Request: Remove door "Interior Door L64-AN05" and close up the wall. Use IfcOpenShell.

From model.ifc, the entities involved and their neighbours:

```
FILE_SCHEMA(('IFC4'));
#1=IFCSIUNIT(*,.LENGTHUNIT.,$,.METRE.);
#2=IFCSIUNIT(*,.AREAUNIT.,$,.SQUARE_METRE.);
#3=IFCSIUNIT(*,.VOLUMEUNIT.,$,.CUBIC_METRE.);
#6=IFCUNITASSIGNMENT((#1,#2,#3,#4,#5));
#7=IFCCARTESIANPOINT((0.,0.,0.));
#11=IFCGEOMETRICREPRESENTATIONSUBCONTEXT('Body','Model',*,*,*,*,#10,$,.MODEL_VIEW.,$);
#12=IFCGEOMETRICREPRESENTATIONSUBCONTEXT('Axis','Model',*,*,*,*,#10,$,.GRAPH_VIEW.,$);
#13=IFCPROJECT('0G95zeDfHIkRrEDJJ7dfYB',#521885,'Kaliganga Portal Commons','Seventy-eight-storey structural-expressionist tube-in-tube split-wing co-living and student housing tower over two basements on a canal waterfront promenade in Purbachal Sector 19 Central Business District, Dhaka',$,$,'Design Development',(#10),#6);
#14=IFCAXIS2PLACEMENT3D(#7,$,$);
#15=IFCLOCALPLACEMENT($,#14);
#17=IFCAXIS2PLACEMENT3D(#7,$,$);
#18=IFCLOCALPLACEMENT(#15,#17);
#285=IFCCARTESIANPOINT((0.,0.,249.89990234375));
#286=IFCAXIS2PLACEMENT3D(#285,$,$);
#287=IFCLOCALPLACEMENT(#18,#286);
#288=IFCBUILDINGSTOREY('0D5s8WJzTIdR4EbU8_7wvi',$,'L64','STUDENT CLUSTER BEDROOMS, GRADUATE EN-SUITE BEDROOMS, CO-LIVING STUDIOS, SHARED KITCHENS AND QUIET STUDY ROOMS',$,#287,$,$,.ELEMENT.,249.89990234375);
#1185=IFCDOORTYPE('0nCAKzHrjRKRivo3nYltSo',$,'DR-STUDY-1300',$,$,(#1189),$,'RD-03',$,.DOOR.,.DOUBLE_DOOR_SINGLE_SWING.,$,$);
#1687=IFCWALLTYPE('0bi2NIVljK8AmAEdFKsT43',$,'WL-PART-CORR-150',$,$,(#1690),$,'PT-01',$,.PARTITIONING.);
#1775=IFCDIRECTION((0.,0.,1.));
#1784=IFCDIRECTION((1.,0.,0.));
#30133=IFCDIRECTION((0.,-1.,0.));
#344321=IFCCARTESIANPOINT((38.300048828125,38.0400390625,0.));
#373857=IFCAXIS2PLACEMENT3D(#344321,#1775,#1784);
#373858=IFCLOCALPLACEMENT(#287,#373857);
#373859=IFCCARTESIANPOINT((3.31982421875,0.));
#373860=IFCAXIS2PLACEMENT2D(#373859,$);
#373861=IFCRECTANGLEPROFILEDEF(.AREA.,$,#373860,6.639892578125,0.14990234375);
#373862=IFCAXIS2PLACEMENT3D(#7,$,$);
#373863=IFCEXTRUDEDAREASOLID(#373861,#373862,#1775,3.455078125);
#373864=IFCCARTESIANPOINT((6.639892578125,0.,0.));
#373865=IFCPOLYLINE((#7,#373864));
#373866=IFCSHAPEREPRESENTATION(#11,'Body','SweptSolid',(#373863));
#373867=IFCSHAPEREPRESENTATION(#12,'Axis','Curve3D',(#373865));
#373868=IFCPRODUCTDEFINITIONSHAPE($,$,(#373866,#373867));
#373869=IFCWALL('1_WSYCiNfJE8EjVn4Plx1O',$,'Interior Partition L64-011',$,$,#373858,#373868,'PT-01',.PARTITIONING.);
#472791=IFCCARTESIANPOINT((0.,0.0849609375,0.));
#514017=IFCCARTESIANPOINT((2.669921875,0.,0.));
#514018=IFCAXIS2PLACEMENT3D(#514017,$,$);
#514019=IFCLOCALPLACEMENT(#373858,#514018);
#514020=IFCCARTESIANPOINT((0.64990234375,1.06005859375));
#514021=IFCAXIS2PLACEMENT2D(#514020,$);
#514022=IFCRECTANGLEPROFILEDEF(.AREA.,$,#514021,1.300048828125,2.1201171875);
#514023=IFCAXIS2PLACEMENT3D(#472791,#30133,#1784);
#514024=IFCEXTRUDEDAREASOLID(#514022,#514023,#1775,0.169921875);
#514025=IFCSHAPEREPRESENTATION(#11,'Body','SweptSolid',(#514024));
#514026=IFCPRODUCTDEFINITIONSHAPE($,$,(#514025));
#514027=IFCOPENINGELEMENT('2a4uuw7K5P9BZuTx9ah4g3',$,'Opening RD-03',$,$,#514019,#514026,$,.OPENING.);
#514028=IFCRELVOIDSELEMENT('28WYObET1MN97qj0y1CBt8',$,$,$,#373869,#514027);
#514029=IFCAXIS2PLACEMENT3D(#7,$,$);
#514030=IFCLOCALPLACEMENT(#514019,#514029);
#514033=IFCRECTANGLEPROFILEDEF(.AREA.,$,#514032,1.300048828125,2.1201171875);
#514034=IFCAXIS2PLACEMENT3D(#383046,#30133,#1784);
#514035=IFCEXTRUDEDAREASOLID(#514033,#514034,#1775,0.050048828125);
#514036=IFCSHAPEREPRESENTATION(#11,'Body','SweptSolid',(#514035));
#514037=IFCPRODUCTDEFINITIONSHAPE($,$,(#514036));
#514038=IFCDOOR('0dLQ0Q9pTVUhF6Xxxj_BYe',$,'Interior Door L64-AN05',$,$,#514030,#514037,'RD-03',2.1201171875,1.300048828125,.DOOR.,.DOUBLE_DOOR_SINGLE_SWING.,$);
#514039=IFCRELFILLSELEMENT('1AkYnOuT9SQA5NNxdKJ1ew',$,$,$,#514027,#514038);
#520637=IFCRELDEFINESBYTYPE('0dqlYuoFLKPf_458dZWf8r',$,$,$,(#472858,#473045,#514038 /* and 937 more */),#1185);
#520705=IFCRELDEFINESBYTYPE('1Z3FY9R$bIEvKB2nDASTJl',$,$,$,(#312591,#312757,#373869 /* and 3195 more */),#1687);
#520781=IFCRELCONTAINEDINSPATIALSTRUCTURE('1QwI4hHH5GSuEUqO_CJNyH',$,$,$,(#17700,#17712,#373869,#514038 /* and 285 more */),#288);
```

```python
import ifcopenshell
import ifcopenshell.api.feature
import ifcopenshell.api.root
import ifcopenshell.geom
import ifcopenshell.util.shape

model = ifcopenshell.open("model.ifc")
settings = ifcopenshell.geom.settings()


def volume(element):
    """Net volume in cubic metres, openings subtracted."""
    shape = ifcopenshell.geom.create_shape(settings, element)
    return ifcopenshell.util.shape.get_volume(shape.geometry)


door = model.by_id(514038)
opening = door.FillsVoids[0].RelatingOpeningElement
wall = opening.VoidsElements[0].RelatingBuildingElement
before = volume(wall)

ifcopenshell.api.root.remove_product(model, product=door)
ifcopenshell.api.feature.remove_feature(model, feature=opening)

after = volume(wall)

print(f"wall volume {before:.3f} -> {after:.3f} m3")

model.write("model_edited.ifc")
```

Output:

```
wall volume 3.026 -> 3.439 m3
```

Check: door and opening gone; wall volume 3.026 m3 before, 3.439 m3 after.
